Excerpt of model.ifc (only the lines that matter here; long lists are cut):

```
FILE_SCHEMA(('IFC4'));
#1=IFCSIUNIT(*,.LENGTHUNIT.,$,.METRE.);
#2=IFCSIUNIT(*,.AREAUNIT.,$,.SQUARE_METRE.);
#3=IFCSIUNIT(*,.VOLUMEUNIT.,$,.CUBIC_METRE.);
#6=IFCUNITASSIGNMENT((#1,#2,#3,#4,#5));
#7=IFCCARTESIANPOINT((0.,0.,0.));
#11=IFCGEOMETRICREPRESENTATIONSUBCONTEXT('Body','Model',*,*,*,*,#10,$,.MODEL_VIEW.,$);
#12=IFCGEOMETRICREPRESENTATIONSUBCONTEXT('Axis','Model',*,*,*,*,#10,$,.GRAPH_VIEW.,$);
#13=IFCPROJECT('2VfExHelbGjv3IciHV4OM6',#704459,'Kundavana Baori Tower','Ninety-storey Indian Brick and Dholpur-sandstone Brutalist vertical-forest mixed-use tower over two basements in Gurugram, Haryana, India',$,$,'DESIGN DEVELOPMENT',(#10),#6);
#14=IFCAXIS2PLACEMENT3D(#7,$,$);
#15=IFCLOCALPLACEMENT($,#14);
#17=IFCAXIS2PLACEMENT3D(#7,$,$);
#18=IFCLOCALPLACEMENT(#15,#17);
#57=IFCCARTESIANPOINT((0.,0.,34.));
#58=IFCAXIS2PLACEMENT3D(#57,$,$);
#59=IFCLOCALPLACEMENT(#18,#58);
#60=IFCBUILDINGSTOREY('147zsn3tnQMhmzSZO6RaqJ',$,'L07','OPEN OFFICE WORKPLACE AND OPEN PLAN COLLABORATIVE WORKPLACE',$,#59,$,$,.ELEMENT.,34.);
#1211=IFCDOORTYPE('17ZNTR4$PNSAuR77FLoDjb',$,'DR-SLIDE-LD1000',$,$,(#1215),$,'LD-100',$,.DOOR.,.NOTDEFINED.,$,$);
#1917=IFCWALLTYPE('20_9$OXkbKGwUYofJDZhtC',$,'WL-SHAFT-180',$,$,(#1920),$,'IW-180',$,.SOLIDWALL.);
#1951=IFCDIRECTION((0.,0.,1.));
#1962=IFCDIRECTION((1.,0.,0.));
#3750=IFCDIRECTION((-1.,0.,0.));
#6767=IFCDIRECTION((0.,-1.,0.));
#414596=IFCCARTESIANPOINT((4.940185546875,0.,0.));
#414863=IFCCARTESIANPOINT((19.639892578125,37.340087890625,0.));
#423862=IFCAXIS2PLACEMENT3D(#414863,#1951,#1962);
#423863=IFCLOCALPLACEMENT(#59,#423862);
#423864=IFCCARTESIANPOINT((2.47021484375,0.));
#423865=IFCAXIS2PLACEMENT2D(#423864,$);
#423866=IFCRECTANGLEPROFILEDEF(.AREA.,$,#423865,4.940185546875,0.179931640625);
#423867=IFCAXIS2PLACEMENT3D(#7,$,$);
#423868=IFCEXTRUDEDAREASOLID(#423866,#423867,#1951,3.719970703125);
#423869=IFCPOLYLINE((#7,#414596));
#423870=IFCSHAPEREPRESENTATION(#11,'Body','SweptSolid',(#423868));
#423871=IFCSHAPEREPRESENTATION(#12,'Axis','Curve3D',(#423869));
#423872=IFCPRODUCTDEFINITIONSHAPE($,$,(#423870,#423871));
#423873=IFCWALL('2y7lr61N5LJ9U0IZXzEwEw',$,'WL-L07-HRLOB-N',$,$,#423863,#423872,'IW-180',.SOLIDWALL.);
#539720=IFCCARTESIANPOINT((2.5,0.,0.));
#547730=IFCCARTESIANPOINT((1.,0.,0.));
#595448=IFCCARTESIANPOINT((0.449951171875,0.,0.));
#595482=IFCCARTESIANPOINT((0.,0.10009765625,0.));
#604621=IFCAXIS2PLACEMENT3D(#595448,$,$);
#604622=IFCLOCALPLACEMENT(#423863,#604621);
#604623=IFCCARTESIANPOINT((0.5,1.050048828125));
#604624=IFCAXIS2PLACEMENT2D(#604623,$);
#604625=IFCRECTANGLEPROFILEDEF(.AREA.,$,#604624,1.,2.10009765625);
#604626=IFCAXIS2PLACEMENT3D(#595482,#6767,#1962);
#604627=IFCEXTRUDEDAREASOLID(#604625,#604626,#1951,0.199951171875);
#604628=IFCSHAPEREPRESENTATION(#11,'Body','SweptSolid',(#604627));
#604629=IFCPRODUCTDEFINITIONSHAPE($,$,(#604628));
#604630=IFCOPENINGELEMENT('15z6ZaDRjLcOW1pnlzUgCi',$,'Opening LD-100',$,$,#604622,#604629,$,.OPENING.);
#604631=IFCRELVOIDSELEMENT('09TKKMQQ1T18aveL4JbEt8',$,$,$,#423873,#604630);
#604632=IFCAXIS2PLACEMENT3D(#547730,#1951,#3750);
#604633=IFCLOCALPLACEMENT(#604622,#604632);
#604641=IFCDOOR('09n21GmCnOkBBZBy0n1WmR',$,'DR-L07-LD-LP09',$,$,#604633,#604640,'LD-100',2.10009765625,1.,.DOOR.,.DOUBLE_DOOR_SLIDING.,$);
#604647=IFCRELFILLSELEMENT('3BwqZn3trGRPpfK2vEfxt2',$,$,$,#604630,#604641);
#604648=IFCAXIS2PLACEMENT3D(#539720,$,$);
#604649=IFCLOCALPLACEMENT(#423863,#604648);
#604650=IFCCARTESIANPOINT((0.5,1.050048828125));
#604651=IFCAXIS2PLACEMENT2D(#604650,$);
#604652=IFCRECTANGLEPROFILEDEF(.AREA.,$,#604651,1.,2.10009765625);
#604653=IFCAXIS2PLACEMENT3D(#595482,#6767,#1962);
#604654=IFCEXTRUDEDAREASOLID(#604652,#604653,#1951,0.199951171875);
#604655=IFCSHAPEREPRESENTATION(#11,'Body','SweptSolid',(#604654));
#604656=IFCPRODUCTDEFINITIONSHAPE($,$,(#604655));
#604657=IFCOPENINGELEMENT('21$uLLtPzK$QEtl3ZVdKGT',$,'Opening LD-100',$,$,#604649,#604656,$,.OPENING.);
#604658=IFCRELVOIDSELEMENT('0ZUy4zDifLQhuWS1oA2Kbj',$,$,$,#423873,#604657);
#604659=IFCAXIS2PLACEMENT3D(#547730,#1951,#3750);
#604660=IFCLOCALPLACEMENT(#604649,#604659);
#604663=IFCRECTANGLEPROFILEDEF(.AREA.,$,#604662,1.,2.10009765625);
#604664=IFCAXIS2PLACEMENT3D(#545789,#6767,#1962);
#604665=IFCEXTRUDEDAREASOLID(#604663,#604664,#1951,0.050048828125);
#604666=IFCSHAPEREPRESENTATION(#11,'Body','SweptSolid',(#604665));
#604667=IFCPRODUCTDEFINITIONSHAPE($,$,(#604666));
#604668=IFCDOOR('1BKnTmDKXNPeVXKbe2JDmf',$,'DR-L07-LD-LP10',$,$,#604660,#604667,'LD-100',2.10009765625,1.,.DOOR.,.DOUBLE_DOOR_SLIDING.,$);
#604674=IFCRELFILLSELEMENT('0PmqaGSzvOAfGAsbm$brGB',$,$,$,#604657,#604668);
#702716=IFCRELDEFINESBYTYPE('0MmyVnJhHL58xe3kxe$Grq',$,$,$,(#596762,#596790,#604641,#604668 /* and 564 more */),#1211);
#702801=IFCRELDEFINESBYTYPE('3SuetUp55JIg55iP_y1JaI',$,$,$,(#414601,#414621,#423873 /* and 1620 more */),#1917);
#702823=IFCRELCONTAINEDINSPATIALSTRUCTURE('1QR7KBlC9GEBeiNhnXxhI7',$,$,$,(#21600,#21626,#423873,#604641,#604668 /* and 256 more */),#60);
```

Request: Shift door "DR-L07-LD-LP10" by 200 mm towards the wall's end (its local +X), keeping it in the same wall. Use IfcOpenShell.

```python
import ifcopenshell
import ifcopenshell.api.geometry
import ifcopenshell.util.placement
import ifcopenshell.util.unit

model = ifcopenshell.open("model.ifc")
unit_scale = ifcopenshell.util.unit.calculate_unit_scale(model)

door = model.by_id(604668)
opening = door.FillsVoids[0].RelatingOpeningElement
wall = opening.VoidsElements[0].RelatingBuildingElement

wall_matrix = ifcopenshell.util.placement.get_local_placement(wall.ObjectPlacement)
shift = wall_matrix[:3, 0] * 0.2 / unit_scale
before = ifcopenshell.util.placement.get_local_placement(door.ObjectPlacement)[:3, 3].copy()

# The door is placed relative to its opening, so it follows when the opening moves.
matrix = ifcopenshell.util.placement.get_local_placement(opening.ObjectPlacement)
matrix[:3, 3] += shift
ifcopenshell.api.geometry.edit_object_placement(
    model, product=opening, matrix=matrix, is_si=False, should_transform_children=True
)

after = ifcopenshell.util.placement.get_local_placement(door.ObjectPlacement)[:3, 3]
print("door moved by", (after - before).round(3) + 0.0)

model.write("model_updated.ifc")
```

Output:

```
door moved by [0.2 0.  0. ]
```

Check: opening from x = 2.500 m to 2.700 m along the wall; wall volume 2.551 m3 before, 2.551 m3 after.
